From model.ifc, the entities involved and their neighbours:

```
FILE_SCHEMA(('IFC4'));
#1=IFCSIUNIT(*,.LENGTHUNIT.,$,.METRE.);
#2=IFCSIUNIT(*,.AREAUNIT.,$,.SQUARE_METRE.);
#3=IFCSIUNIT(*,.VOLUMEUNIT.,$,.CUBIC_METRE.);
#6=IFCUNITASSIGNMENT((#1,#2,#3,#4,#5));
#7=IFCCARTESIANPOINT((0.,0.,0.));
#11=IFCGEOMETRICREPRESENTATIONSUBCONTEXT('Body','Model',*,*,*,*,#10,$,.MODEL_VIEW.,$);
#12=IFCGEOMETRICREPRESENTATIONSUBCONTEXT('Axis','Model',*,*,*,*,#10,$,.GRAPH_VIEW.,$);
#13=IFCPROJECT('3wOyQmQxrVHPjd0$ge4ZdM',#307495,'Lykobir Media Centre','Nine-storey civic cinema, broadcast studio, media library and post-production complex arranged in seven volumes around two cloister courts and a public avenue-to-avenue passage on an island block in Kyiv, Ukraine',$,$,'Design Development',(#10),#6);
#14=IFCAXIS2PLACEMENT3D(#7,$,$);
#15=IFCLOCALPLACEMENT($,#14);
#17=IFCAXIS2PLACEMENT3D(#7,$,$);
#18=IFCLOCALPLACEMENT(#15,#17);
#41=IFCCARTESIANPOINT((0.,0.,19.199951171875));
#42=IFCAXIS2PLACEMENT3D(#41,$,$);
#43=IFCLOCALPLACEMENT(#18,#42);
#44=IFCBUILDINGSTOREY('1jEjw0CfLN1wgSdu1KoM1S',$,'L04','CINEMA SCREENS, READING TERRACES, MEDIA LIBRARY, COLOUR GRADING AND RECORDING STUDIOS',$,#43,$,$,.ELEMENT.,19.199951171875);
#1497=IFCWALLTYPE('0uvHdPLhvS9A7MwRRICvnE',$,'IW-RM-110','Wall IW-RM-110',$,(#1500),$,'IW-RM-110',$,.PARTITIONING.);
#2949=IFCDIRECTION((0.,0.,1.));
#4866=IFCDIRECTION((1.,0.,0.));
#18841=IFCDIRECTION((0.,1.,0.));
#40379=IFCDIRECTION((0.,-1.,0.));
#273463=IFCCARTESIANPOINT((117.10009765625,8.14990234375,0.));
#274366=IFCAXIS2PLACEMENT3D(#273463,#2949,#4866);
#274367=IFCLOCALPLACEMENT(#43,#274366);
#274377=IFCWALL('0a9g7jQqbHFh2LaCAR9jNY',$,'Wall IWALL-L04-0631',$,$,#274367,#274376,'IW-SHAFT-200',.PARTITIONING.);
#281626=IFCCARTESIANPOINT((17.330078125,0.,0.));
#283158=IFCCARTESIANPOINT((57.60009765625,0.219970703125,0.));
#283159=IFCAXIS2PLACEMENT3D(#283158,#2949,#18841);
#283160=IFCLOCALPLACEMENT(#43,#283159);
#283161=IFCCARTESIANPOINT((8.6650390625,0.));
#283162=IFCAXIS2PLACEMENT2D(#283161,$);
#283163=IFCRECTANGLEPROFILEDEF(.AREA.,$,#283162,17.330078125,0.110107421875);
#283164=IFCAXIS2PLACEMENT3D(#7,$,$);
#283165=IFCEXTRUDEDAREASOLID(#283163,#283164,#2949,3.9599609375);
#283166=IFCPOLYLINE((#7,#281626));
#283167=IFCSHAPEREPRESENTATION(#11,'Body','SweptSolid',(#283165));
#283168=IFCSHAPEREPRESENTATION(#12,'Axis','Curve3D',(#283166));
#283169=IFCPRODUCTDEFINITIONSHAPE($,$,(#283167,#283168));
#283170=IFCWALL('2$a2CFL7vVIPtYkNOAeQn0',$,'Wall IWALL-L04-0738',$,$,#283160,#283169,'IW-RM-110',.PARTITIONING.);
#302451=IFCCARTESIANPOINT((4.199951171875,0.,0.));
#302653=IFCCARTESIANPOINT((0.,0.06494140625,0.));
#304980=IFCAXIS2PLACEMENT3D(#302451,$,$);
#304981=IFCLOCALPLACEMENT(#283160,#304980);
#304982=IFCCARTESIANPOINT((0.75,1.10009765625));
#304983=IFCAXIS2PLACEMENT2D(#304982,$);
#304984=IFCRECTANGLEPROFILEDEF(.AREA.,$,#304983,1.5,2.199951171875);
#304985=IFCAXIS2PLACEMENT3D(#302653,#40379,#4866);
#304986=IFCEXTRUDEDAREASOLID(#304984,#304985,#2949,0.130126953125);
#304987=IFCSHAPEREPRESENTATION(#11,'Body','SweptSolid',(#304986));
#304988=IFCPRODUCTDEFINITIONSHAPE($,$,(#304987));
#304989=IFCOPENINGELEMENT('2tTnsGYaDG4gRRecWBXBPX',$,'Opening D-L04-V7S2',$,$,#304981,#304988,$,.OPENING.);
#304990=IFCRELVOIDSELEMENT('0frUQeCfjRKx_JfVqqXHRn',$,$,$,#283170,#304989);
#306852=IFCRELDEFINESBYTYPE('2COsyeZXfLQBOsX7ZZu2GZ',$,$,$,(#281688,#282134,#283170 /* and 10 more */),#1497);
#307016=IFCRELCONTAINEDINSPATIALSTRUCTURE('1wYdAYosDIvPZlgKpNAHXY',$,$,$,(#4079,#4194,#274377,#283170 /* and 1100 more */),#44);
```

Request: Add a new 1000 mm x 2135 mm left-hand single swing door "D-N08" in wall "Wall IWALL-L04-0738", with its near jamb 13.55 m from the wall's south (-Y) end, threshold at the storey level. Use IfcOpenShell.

```python
import numpy as np
import ifcopenshell
import ifcopenshell.api.feature
import ifcopenshell.api.geometry
import ifcopenshell.api.root
import ifcopenshell.api.spatial
import ifcopenshell.geom
import ifcopenshell.util.element
import ifcopenshell.util.placement
import ifcopenshell.util.representation
import ifcopenshell.util.shape
import ifcopenshell.util.unit

model = ifcopenshell.open("model.ifc")
unit_scale = ifcopenshell.util.unit.calculate_unit_scale(model)
settings = ifcopenshell.geom.settings()


def volume(element):
    """Net volume in cubic metres, openings subtracted."""
    shape = ifcopenshell.geom.create_shape(settings, element)
    return ifcopenshell.util.shape.get_volume(shape.geometry)


wall = model.by_id(283170)
storey = ifcopenshell.util.element.get_container(wall, ifc_class="IfcBuildingStorey")
context = ifcopenshell.util.representation.get_context(model, "Model", "Body", "MODEL_VIEW")
before = volume(wall)

width, height, from_end, sill = 1, 2.135, 13.55, 0.0  # metres

# The wall runs along its own X axis, and the end named is its -X end.
wall_shape = ifcopenshell.geom.create_shape(settings, wall)
x, y, z = ifcopenshell.util.shape.get_vertices(wall_shape.geometry).T
start = x.min() + from_end
face, thickness = float(y.min()), float(y.max() - y.min())
wall_matrix = ifcopenshell.util.placement.get_local_placement(wall.ObjectPlacement)
level = ifcopenshell.util.placement.get_local_placement(storey.ObjectPlacement)[2, 3]


def in_wall(x, y):
    """Placement at x, y metres in the wall's axes, at sill height."""
    matrix = wall_matrix.copy()
    matrix[:, 3] = wall_matrix @ np.array([x / unit_scale, y / unit_scale, 0.0, 1.0])
    matrix[2, 3] = level + sill / unit_scale
    return matrix


# Opening: a box that overshoots both wall faces by 50 mm.
opening = ifcopenshell.api.root.create_entity(model, ifc_class="IfcOpeningElement", predefined_type="OPENING")
box = ifcopenshell.api.geometry.add_wall_representation(
    model, context=context, length=width, height=height, thickness=thickness + 0.1
)
ifcopenshell.api.geometry.assign_representation(model, product=opening, representation=box)
ifcopenshell.api.geometry.edit_object_placement(model, product=opening, matrix=in_wall(start, face - 0.05), is_si=False)
ifcopenshell.api.feature.add_feature(model, feature=opening, element=wall)

door = ifcopenshell.api.root.create_entity(model, ifc_class="IfcDoor", name="D-N08", predefined_type="DOOR")
door.OverallWidth, door.OverallHeight = width / unit_scale, height / unit_scale
door.OperationType = "SINGLE_SWING_LEFT"
body = ifcopenshell.api.geometry.add_door_representation(
    model,
    context=context,
    overall_width=door.OverallWidth,
    overall_height=door.OverallHeight,
    operation_type="SINGLE_SWING_LEFT",
    lining_properties={"LiningDepth": thickness / unit_scale, "ThresholdDepth": thickness / unit_scale},
)
ifcopenshell.api.geometry.assign_representation(model, product=door, representation=body)
ifcopenshell.api.spatial.assign_container(model, products=[door], relating_structure=storey)
ifcopenshell.api.feature.add_filling(model, opening=opening, element=door)

# The lining spans the wall, so the door starts at the wall face.
ifcopenshell.api.geometry.edit_object_placement(model, product=door, matrix=in_wall(start, face), is_si=False)

after = volume(wall)

print(f"wall volume {before:.3f} -> {after:.3f} m3")

model.write("model_rev.ifc")
```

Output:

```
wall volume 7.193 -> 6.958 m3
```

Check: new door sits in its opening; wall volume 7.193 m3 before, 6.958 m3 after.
